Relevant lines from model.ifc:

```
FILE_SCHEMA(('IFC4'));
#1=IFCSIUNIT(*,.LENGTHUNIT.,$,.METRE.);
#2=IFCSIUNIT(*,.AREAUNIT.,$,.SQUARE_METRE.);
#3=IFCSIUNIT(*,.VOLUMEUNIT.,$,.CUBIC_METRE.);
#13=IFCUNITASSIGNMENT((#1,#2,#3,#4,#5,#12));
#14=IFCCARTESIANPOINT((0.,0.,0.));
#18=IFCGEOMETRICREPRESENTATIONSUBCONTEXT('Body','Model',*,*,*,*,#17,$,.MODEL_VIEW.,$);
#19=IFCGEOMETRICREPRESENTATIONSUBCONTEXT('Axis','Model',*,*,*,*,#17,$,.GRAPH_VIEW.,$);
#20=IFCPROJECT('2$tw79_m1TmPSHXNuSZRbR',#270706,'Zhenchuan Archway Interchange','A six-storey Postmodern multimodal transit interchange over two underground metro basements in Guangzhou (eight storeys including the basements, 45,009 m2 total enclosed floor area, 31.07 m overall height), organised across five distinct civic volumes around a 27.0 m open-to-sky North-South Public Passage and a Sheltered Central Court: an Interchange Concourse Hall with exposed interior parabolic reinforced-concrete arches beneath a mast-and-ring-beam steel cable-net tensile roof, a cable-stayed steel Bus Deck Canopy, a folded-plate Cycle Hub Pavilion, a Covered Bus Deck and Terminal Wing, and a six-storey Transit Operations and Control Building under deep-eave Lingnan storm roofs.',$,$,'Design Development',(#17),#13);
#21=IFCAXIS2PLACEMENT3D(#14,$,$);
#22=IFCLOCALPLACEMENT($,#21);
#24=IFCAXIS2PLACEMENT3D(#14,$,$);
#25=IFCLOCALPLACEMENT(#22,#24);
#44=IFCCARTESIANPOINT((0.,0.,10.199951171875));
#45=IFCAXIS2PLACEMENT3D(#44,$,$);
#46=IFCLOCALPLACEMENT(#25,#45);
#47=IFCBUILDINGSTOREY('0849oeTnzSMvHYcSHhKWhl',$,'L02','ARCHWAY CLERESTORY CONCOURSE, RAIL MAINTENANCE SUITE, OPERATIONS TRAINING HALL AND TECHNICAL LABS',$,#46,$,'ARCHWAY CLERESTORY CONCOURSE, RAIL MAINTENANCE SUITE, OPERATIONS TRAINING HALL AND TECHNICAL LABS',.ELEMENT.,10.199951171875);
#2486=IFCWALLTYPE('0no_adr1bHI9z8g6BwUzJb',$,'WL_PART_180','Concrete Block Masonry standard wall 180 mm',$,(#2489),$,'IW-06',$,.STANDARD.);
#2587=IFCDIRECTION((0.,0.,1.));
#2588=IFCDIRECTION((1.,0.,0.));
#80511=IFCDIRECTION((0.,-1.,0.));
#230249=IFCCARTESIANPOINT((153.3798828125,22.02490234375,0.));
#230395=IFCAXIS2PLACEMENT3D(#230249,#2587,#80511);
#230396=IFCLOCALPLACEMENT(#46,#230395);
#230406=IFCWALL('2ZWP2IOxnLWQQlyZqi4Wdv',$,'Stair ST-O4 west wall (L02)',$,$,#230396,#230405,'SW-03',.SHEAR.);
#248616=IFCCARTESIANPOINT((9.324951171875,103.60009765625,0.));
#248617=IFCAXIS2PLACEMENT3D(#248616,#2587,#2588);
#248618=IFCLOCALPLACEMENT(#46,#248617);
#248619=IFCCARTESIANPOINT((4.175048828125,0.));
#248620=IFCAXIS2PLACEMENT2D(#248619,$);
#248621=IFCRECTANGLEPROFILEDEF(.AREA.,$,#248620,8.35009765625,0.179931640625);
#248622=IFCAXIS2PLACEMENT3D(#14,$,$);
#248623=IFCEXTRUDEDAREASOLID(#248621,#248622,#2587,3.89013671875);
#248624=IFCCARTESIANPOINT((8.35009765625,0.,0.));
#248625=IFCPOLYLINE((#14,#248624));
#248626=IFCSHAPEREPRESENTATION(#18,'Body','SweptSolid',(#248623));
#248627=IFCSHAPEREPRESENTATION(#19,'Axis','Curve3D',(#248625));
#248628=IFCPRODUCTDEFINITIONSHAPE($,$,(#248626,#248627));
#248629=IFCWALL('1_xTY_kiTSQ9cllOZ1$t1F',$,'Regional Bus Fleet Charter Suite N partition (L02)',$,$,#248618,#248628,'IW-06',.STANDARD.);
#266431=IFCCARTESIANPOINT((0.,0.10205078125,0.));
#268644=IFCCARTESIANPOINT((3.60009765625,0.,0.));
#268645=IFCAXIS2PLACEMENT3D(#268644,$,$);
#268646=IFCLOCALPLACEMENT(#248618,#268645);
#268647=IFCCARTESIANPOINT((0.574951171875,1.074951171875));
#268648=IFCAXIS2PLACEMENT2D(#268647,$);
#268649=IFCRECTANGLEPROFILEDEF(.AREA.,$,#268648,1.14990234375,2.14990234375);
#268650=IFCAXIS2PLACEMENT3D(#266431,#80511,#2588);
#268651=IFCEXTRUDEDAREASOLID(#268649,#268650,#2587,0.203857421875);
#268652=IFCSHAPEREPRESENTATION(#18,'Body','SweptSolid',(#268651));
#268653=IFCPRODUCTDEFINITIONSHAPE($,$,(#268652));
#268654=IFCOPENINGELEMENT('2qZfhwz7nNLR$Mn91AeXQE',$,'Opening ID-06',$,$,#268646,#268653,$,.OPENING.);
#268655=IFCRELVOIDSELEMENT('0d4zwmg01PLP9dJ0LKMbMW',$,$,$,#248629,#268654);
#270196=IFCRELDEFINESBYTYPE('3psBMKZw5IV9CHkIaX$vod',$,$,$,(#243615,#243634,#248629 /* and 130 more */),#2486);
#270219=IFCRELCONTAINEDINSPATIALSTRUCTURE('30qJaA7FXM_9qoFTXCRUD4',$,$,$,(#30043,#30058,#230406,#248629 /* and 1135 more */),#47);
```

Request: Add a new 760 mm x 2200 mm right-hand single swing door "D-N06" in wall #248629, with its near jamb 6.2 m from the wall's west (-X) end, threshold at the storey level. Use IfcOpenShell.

```python
import numpy as np
import ifcopenshell
import ifcopenshell.api.feature
import ifcopenshell.api.geometry
import ifcopenshell.api.root
import ifcopenshell.api.spatial
import ifcopenshell.geom
import ifcopenshell.util.element
import ifcopenshell.util.placement
import ifcopenshell.util.representation
import ifcopenshell.util.shape
import ifcopenshell.util.unit

model = ifcopenshell.open("model.ifc")
unit_scale = ifcopenshell.util.unit.calculate_unit_scale(model)
settings = ifcopenshell.geom.settings()


def volume(element):
    """Net volume in cubic metres, openings subtracted."""
    shape = ifcopenshell.geom.create_shape(settings, element)
    return ifcopenshell.util.shape.get_volume(shape.geometry)


wall = model.by_guid("1_xTY_kiTSQ9cllOZ1$t1F")
storey = ifcopenshell.util.element.get_container(wall, ifc_class="IfcBuildingStorey")
context = ifcopenshell.util.representation.get_context(model, "Model", "Body", "MODEL_VIEW")
before = volume(wall)

width, height, from_end, sill = 0.76, 2.2, 6.2, 0.0  # metres

# The wall runs along its own X axis, and the end named is its -X end.
wall_shape = ifcopenshell.geom.create_shape(settings, wall)
x, y, z = ifcopenshell.util.shape.get_vertices(wall_shape.geometry).T
start = x.min() + from_end
face, thickness = float(y.min()), float(y.max() - y.min())
wall_matrix = ifcopenshell.util.placement.get_local_placement(wall.ObjectPlacement)
level = ifcopenshell.util.placement.get_local_placement(storey.ObjectPlacement)[2, 3]


def in_wall(x, y):
    """Placement at x, y metres in the wall's axes, at sill height."""
    matrix = wall_matrix.copy()
    matrix[:, 3] = wall_matrix @ np.array([x / unit_scale, y / unit_scale, 0.0, 1.0])
    matrix[2, 3] = level + sill / unit_scale
    return matrix


# Opening: a box that overshoots both wall faces by 50 mm.
opening = ifcopenshell.api.root.create_entity(model, ifc_class="IfcOpeningElement", predefined_type="OPENING")
box = ifcopenshell.api.geometry.add_wall_representation(
    model, context=context, length=width, height=height, thickness=thickness + 0.1
)
ifcopenshell.api.geometry.assign_representation(model, product=opening, representation=box)
ifcopenshell.api.geometry.edit_object_placement(model, product=opening, matrix=in_wall(start, face - 0.05), is_si=False)
ifcopenshell.api.feature.add_feature(model, feature=opening, element=wall)

door = ifcopenshell.api.root.create_entity(model, ifc_class="IfcDoor", name="D-N06", predefined_type="DOOR")
door.OverallWidth, door.OverallHeight = width / unit_scale, height / unit_scale
door.OperationType = "SINGLE_SWING_RIGHT"
body = ifcopenshell.api.geometry.add_door_representation(
    model,
    context=context,
    overall_width=door.OverallWidth,
    overall_height=door.OverallHeight,
    operation_type="SINGLE_SWING_RIGHT",
    lining_properties={"LiningDepth": thickness / unit_scale, "ThresholdDepth": thickness / unit_scale},
)
ifcopenshell.api.geometry.assign_representation(model, product=door, representation=body)
ifcopenshell.api.spatial.assign_container(model, products=[door], relating_structure=storey)
ifcopenshell.api.feature.add_filling(model, opening=opening, element=door)

# The lining spans the wall, so the door starts at the wall face.
ifcopenshell.api.geometry.edit_object_placement(model, product=door, matrix=in_wall(start, face), is_si=False)

after = volume(wall)

print(f"wall volume {before:.3f} -> {after:.3f} m3")

model.write("model_v2.ifc")
```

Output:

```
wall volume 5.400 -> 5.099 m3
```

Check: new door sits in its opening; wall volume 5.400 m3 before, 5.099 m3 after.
